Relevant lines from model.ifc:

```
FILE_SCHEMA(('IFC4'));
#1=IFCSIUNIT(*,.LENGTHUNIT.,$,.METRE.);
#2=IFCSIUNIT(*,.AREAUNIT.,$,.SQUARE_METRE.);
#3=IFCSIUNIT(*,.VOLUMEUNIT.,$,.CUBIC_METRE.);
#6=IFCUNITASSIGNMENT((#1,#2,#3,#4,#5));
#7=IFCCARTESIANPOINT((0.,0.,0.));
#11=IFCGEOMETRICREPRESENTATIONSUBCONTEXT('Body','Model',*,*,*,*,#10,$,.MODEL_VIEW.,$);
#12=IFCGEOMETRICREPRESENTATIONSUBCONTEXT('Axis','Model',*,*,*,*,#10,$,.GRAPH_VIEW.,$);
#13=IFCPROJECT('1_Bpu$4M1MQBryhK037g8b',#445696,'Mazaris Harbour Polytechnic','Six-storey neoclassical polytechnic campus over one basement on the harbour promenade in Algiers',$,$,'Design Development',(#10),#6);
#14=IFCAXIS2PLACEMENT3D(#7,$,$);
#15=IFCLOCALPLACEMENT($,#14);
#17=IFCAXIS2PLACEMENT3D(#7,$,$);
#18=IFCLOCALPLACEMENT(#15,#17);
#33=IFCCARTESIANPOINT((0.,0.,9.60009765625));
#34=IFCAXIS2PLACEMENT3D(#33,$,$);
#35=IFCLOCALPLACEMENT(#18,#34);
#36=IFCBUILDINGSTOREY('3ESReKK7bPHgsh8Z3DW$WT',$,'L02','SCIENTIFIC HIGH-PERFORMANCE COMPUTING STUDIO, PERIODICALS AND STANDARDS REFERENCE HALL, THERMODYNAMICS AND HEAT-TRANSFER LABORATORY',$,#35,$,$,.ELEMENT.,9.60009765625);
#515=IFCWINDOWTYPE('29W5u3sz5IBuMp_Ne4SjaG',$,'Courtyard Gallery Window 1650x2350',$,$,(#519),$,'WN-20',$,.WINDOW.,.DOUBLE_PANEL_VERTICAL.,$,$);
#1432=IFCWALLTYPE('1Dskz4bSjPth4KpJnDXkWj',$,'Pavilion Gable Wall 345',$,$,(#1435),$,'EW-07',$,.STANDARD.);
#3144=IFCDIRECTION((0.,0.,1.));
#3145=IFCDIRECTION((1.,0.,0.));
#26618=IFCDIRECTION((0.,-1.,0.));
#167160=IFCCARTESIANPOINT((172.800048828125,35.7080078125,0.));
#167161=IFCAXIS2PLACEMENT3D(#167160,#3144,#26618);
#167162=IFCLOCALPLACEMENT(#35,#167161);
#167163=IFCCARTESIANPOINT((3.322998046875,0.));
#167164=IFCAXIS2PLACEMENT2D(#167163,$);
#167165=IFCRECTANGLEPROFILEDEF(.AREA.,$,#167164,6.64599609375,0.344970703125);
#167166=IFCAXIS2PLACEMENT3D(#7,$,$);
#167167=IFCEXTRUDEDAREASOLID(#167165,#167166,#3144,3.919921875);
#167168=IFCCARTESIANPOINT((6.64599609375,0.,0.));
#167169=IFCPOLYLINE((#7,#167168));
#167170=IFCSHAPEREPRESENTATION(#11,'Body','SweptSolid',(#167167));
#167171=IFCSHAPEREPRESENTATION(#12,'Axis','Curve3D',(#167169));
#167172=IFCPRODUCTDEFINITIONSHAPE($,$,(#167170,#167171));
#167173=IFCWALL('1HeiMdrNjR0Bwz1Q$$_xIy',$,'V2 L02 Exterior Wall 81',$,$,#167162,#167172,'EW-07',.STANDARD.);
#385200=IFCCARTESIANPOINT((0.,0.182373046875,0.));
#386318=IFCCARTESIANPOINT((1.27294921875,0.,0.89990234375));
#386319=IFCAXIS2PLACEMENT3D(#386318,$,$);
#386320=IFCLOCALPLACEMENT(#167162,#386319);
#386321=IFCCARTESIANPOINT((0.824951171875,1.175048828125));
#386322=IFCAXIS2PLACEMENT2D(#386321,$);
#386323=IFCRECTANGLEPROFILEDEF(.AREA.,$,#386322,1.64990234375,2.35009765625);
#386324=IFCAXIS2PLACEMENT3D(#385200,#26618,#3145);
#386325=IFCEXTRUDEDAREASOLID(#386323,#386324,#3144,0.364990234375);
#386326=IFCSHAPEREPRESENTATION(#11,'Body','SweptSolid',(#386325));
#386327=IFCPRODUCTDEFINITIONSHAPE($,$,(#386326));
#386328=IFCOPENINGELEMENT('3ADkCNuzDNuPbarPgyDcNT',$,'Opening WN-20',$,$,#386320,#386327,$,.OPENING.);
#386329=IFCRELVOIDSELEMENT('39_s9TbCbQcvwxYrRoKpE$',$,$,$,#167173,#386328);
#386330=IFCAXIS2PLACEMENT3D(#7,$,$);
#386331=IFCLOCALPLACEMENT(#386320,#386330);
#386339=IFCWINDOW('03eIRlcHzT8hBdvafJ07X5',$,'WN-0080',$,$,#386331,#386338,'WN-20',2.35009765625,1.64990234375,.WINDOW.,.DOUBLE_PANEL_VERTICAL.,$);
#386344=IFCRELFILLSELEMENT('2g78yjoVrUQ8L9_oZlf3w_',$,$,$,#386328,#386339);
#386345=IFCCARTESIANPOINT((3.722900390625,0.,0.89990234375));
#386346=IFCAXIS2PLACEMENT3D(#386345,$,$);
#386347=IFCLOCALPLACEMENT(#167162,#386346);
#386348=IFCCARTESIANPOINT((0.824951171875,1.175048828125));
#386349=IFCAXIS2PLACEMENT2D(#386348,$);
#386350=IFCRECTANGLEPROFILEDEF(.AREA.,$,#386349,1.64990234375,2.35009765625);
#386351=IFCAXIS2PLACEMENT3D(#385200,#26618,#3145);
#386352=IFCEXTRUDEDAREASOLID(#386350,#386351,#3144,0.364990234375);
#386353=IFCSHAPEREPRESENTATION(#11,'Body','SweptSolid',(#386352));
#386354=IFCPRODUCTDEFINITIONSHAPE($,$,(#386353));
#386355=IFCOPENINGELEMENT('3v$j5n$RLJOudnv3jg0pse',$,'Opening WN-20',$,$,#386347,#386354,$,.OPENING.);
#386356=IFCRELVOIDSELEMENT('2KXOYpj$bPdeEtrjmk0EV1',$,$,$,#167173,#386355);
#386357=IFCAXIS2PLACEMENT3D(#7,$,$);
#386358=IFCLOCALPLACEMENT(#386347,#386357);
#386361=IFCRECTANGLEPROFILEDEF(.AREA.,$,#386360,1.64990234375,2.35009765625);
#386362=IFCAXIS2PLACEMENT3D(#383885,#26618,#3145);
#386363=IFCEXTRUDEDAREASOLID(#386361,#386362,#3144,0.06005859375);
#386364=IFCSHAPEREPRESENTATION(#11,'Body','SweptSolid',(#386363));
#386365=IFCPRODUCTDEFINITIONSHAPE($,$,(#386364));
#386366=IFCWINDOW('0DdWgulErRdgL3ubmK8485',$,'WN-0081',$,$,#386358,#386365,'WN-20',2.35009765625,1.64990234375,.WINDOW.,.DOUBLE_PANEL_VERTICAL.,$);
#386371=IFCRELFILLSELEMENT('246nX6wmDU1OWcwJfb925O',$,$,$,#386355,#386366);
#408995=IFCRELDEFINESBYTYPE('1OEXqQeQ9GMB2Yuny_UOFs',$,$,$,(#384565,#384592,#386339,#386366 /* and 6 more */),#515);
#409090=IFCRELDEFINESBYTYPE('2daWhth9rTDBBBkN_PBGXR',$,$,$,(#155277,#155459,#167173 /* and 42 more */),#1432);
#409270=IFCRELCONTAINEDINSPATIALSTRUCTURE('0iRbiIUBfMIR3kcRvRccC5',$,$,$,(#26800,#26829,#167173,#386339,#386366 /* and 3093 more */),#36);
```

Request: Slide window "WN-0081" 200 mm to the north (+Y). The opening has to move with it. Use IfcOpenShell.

```python
import ifcopenshell
import ifcopenshell.api.geometry
import ifcopenshell.util.placement
import ifcopenshell.util.unit

model = ifcopenshell.open("model.ifc")
unit_scale = ifcopenshell.util.unit.calculate_unit_scale(model)

window = model.by_guid("0DdWgulErRdgL3ubmK8485")
opening = window.FillsVoids[0].RelatingOpeningElement
wall = opening.VoidsElements[0].RelatingBuildingElement

wall_matrix = ifcopenshell.util.placement.get_local_placement(wall.ObjectPlacement)
shift = wall_matrix[:3, 0] * -0.2 / unit_scale
before = ifcopenshell.util.placement.get_local_placement(window.ObjectPlacement)[:3, 3].copy()

# The window is placed relative to its opening, so it follows when the opening moves.
matrix = ifcopenshell.util.placement.get_local_placement(opening.ObjectPlacement)
matrix[:3, 3] += shift
ifcopenshell.api.geometry.edit_object_placement(
    model, product=opening, matrix=matrix, is_si=False, should_transform_children=True
)

after = ifcopenshell.util.placement.get_local_placement(window.ObjectPlacement)[:3, 3]
print("window moved by", (after - before).round(3) + 0.0)

model.write("model_v2.ifc")
```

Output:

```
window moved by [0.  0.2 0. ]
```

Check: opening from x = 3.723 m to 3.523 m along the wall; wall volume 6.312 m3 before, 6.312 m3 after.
